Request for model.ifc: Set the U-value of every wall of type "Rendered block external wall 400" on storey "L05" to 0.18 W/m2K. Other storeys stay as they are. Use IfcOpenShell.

First a look at what the model holds.

```python
import ifcopenshell
import ifcopenshell.util.element

model = ifcopenshell.open("model.ifc")
print(model.schema)
storey = next(s for s in model.by_type("IfcBuildingStorey") if s.Name == "L05")
walls = [e for e in ifcopenshell.util.element.get_decomposition(storey) if e.is_a("IfcWall")]
seen = {}
for e in walls:
    element_type = ifcopenshell.util.element.get_type(e)
    key = (element_type.Name if element_type != e and element_type else None, ifcopenshell.util.element.get_pset(e, "Pset_WallCommon", "ThermalTransmittance"))
    seen[key] = seen.get(key, 0) + 1
for (name, value), count in sorted(seen.items(), key=str):
    print(count, "x", name, "|", value)
```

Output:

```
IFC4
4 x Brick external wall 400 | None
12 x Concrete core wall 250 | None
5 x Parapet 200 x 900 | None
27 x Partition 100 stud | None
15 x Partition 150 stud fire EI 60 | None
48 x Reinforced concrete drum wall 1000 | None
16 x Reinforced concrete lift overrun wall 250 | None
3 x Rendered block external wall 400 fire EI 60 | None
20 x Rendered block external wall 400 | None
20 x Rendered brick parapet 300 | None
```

```python
import ifcopenshell
import ifcopenshell.api.pset
import ifcopenshell.util.element

model = ifcopenshell.open("model.ifc")

storey = next(s for s in model.by_type("IfcBuildingStorey") if s.Name == "L05")
walls = [e for e in ifcopenshell.util.element.get_decomposition(storey) if e.is_a("IfcWall")]

count = 0
for e in walls:
    element_type = ifcopenshell.util.element.get_type(e)
    if element_type in (None, e) or element_type.Name != "Rendered block external wall 400":
        continue
    # add_pset returns the element's existing set when there is one.
    pset = ifcopenshell.api.pset.add_pset(model, product=e, name="Pset_WallCommon")
    ifcopenshell.api.pset.edit_pset(model, pset=pset, properties={"ThermalTransmittance": 0.18})
    count += 1

print(count, "walls updated")

model.write("model_v2.ifc")
```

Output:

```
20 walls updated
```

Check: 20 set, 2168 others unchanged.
